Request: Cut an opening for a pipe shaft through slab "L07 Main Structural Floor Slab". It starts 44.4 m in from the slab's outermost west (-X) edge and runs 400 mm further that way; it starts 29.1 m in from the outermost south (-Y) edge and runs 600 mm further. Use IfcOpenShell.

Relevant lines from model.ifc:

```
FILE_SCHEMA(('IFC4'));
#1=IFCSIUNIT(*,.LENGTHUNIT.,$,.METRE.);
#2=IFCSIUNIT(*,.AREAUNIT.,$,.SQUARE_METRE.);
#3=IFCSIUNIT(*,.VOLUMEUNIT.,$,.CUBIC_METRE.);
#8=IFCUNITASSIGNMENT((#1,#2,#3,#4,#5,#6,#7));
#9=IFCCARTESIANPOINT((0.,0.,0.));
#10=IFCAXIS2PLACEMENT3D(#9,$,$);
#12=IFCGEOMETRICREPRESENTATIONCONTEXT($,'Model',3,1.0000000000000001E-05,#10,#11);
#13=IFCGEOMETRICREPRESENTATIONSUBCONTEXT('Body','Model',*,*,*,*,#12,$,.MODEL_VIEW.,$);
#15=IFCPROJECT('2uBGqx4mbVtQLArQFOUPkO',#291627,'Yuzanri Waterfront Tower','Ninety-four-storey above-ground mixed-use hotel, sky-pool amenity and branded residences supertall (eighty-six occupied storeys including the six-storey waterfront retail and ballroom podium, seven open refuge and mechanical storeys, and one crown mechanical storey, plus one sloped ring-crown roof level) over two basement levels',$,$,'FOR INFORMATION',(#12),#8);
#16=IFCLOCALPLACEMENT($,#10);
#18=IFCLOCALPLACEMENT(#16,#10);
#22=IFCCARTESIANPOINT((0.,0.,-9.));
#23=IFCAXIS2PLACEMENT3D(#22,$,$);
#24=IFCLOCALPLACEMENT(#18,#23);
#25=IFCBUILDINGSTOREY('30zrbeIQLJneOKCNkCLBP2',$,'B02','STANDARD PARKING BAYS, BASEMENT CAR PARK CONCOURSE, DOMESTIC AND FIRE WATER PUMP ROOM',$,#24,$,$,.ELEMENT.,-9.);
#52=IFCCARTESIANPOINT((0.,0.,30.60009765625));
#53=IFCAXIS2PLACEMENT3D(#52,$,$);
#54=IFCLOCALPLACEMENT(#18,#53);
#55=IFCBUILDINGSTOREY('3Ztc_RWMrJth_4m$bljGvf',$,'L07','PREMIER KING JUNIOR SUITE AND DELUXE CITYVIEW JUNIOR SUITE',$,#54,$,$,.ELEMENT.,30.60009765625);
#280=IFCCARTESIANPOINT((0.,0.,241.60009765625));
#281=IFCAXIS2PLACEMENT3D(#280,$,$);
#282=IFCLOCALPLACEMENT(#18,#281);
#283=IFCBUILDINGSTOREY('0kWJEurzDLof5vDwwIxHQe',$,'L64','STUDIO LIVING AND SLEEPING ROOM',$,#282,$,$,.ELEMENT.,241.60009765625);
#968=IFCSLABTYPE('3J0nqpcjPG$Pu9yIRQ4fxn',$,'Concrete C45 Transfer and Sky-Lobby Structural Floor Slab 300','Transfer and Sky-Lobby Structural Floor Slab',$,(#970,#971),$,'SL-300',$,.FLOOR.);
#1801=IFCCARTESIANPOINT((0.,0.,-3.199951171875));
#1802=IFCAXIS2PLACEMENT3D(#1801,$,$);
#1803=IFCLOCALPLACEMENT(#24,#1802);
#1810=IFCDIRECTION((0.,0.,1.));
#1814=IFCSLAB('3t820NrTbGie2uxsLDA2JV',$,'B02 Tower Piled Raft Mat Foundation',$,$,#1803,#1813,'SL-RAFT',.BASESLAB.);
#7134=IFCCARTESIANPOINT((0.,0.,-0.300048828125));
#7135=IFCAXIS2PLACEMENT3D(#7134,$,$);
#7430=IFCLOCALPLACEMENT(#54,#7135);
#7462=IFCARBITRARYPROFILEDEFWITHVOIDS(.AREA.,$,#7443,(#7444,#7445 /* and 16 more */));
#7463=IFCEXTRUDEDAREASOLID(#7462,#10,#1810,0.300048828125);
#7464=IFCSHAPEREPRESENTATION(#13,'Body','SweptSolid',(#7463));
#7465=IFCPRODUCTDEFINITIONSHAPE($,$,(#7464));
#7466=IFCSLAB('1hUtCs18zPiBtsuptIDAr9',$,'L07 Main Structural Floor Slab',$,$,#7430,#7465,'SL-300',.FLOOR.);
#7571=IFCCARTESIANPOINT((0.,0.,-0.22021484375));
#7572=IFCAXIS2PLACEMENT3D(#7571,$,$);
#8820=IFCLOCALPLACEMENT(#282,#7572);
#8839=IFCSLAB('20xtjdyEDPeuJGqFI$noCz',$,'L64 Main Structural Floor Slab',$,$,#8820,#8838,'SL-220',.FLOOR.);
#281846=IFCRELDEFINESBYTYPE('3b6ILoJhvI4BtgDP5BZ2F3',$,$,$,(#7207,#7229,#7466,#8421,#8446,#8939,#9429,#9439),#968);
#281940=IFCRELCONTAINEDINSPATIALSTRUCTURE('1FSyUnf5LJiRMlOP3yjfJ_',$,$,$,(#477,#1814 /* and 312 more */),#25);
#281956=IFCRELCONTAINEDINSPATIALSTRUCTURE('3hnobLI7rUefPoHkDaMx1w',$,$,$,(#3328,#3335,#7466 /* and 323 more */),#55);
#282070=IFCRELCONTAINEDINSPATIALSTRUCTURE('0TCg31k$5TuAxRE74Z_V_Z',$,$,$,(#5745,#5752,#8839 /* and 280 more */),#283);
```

```python
import numpy as np
import ifcopenshell
import ifcopenshell.api.feature
import ifcopenshell.api.geometry
import ifcopenshell.api.root
import ifcopenshell.geom
import ifcopenshell.util.placement
import ifcopenshell.util.representation
import ifcopenshell.util.shape
import ifcopenshell.util.unit

model = ifcopenshell.open("model.ifc")
unit_scale = ifcopenshell.util.unit.calculate_unit_scale(model)
settings = ifcopenshell.geom.settings()


def volume(element):
    """Net volume in cubic metres, openings subtracted."""
    shape = ifcopenshell.geom.create_shape(settings, element)
    return ifcopenshell.util.shape.get_volume(shape.geometry)


slab = model.by_id(7466)
before = volume(slab)

# Extent in the slab's own axes, in metres. The edges named are its -X and -Y sides.
slab_shape = ifcopenshell.geom.create_shape(settings, slab)
vertices = ifcopenshell.util.shape.get_vertices(slab_shape.geometry)
x_min, y_min, bottom = vertices.min(axis=0)
top = vertices[:, 2].max()

opening = ifcopenshell.api.root.create_entity(model, ifc_class="IfcOpeningElement", name="Pipe shaft opening", predefined_type="OPENING")
context = ifcopenshell.util.representation.get_context(model, "Model", "Body", "MODEL_VIEW")
width, depth = 0.4, 0.6
outline = [(0.0, 0.0), (width, 0.0), (width, depth), (0.0, depth), (0.0, 0.0)]
# Overshoot both faces by 50 mm so the cut is clean.
shape = ifcopenshell.api.geometry.add_slab_representation(
    model, context=context, depth=top - bottom + 0.1, polyline=outline
)
ifcopenshell.api.geometry.assign_representation(model, product=opening, representation=shape)

matrix = ifcopenshell.util.placement.get_local_placement(slab.ObjectPlacement)
matrix[:, 3] = matrix @ np.append(np.array([x_min + 44.4, y_min + 29.1, bottom - 0.05]) / unit_scale, 1.0)
ifcopenshell.api.geometry.edit_object_placement(model, product=opening, matrix=matrix, is_si=False)
ifcopenshell.api.feature.add_feature(model, feature=opening, element=slab)

after = volume(slab)

print(f"slab volume {before:.3f} -> {after:.3f} m3")

model.write("model_edited.ifc")
```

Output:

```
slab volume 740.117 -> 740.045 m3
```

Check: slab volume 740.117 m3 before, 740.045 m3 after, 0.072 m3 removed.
